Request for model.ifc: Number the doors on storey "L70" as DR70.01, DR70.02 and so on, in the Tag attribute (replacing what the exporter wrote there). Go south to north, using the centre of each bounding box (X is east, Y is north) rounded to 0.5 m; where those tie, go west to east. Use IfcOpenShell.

First a look at what the model holds.

```python
import ifcopenshell
import ifcopenshell.util.element
import ifcopenshell.util.placement

model = ifcopenshell.open("model.ifc")
print(model.schema)
storey = next(s for s in model.by_type("IfcBuildingStorey") if s.Name == "L70")
doors = [e for e in ifcopenshell.util.element.get_decomposition(storey) if e.is_a("IfcDoor")]
for e in sorted(doors, key=lambda e: e.id()):
    origin = ifcopenshell.util.placement.get_local_placement(e.ObjectPlacement)[:3, 3]
    print(e.id(), e.Tag, e.Name, origin.round(2) + 0.0, sep=" | ")
```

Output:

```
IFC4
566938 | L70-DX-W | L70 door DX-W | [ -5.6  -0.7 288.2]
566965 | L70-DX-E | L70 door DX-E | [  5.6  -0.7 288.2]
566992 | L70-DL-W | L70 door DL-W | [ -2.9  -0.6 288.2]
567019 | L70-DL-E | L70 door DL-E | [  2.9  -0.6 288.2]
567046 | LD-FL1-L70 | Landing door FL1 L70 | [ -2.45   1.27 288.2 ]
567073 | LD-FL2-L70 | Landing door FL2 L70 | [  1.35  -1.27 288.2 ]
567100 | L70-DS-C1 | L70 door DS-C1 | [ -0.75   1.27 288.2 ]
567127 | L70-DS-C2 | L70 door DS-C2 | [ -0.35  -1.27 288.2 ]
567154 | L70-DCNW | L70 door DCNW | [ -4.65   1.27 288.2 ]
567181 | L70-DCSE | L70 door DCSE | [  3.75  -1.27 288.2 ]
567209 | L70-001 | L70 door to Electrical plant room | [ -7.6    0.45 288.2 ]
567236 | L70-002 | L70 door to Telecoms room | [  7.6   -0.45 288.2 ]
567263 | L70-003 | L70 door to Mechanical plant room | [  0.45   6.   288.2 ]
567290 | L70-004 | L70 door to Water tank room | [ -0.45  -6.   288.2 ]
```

```python
import ifcopenshell
import ifcopenshell.geom
import ifcopenshell.util.element
import ifcopenshell.util.shape

model = ifcopenshell.open("model.ifc")
settings = ifcopenshell.geom.settings()
settings.set("use-world-coords", True)


def centre(element):
    shape = ifcopenshell.geom.create_shape(settings, element)
    return ifcopenshell.util.shape.get_bbox_centroid(shape.geometry)


storey = next(s for s in model.by_type("IfcBuildingStorey") if s.Name == "L70")
doors = [e for e in ifcopenshell.util.element.get_decomposition(storey) if e.is_a("IfcDoor")]

# Insertion points can sit at a corner or the storey origin, so sort by the geometry (in metres).
centres = {e: centre(e) for e in doors}
doors.sort(key=lambda e: (round(centres[e][1] / 0.5), centres[e][0]))

for i, e in enumerate(doors, start=1):
    number = f"DR70.{i:02d}"
    e.Tag = number
    print(e.id(), number)

model.write("model_edited.ifc")
```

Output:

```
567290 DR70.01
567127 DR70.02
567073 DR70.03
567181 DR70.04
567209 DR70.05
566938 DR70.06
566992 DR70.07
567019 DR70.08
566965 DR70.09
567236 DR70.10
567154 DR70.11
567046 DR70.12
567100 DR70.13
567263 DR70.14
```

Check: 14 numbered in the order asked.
